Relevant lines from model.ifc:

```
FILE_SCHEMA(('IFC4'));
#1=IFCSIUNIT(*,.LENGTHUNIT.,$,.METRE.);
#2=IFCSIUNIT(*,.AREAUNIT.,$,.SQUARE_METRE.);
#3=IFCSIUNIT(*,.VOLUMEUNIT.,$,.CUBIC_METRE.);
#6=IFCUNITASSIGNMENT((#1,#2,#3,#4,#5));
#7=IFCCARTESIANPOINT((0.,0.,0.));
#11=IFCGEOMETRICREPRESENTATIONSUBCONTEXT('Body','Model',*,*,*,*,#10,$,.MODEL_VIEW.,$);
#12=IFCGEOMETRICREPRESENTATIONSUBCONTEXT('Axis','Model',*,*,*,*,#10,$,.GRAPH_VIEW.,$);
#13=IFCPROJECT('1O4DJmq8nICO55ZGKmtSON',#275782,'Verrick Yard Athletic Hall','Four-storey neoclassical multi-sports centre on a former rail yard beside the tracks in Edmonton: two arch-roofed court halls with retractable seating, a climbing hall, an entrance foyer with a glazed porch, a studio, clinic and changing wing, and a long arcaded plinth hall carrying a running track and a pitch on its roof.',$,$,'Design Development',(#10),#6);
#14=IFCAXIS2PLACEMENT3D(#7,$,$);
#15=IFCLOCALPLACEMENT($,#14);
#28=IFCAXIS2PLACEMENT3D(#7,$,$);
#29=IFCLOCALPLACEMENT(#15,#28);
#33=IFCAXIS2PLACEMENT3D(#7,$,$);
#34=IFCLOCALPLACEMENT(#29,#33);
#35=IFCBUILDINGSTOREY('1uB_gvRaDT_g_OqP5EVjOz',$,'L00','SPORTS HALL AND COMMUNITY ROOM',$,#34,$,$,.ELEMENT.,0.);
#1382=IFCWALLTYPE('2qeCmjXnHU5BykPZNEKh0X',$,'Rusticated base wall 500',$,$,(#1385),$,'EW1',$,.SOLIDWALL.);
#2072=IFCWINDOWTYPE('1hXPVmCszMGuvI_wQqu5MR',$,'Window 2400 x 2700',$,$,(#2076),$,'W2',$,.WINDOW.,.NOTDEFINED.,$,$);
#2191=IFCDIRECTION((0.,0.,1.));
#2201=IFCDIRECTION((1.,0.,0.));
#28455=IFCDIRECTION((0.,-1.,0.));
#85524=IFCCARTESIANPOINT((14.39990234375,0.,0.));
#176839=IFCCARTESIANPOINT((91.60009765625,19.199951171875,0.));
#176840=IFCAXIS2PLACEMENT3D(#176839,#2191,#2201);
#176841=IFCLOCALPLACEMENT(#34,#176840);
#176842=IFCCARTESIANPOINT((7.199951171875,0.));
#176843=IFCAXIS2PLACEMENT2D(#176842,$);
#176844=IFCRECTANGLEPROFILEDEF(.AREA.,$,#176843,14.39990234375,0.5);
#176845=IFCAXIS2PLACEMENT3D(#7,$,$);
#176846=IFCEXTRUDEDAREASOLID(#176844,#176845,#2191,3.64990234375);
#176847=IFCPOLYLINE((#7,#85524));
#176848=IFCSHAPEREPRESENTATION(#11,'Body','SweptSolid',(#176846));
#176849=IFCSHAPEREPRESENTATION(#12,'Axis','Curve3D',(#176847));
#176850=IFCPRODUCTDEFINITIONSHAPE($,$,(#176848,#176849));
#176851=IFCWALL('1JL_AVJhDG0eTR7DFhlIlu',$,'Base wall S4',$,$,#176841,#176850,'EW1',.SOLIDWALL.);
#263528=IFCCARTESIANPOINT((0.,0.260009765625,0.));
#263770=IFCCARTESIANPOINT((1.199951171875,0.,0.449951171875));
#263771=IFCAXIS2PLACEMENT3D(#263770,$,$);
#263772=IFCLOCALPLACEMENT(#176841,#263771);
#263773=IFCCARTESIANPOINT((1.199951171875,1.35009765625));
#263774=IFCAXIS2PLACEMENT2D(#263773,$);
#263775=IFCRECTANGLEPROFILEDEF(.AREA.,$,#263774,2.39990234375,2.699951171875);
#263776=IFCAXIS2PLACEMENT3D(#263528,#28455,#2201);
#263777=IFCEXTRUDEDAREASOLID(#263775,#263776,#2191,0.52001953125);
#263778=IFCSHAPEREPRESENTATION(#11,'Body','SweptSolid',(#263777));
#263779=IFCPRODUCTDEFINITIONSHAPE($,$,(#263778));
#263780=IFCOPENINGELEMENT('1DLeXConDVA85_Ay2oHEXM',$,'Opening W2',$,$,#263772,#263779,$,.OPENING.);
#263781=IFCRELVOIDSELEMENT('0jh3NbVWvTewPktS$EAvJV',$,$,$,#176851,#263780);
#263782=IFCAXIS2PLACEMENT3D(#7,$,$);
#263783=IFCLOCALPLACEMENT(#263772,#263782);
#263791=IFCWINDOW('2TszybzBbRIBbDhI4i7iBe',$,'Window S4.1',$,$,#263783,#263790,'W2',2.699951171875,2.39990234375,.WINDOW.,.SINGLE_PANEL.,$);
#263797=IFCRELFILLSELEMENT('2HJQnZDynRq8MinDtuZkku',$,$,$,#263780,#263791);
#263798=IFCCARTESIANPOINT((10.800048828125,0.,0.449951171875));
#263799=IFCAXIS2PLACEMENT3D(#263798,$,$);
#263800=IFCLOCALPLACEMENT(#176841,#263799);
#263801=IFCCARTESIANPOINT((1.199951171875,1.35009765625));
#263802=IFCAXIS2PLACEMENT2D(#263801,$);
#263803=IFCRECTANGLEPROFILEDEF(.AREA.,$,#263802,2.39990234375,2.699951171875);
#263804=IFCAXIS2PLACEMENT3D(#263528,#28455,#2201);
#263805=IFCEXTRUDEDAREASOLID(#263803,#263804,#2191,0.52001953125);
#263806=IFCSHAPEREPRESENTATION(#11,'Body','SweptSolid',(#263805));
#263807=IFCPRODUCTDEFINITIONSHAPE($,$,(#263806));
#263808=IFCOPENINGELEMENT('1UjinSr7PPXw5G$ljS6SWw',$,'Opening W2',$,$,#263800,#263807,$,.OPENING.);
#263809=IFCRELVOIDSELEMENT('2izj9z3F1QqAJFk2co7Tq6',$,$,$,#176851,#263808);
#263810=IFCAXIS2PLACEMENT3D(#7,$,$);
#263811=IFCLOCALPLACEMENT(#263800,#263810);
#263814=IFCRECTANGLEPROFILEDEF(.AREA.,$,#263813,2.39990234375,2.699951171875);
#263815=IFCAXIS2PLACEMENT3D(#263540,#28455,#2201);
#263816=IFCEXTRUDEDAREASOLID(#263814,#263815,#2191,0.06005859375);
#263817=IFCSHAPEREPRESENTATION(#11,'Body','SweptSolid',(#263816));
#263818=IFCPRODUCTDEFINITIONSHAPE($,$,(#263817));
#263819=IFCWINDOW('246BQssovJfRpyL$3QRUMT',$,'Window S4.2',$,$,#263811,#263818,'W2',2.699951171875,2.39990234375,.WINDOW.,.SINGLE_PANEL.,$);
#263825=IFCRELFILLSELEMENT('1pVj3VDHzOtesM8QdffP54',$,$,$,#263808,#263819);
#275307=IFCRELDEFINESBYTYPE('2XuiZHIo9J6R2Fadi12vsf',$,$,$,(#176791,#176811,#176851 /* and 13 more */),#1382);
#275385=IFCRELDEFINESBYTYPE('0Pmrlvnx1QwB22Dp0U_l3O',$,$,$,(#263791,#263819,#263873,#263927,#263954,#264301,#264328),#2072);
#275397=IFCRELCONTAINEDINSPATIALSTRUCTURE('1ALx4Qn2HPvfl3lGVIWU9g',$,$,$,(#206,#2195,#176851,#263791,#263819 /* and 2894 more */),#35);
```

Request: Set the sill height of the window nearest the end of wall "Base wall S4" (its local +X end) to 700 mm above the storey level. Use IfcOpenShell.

```python
import numpy as np
import ifcopenshell
import ifcopenshell.api.geometry
import ifcopenshell.geom
import ifcopenshell.util.element
import ifcopenshell.util.placement
import ifcopenshell.util.shape
import ifcopenshell.util.unit

model = ifcopenshell.open("model.ifc")
unit_scale = ifcopenshell.util.unit.calculate_unit_scale(model)

window = model.by_guid("246BQssovJfRpyL$3QRUMT")
opening = window.FillsVoids[0].RelatingOpeningElement
storey = ifcopenshell.util.element.get_container(window, ifc_class="IfcBuildingStorey")
level = ifcopenshell.util.placement.get_local_placement(storey.ObjectPlacement)[2, 3]

# The opening's origin need not be at the sill, so measure its lowest point.
shape = ifcopenshell.geom.create_shape(ifcopenshell.geom.settings(), opening)
bottom = ifcopenshell.util.shape.get_shape_bottom_elevation(shape, shape.geometry) / unit_scale
dz = level + 0.7 / unit_scale - bottom

shift = np.array([0.0, 0.0, dz])
# The window is placed relative to its opening, so it follows when the opening moves.
matrix = ifcopenshell.util.placement.get_local_placement(opening.ObjectPlacement)
matrix[:3, 3] += shift
ifcopenshell.api.geometry.edit_object_placement(
    model, product=opening, matrix=matrix, is_si=False, should_transform_children=True
)

print(f"moved by {dz * unit_scale:+.3f} m")

model.write("model_v2.ifc")
```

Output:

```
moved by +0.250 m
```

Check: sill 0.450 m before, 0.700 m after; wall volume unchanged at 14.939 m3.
